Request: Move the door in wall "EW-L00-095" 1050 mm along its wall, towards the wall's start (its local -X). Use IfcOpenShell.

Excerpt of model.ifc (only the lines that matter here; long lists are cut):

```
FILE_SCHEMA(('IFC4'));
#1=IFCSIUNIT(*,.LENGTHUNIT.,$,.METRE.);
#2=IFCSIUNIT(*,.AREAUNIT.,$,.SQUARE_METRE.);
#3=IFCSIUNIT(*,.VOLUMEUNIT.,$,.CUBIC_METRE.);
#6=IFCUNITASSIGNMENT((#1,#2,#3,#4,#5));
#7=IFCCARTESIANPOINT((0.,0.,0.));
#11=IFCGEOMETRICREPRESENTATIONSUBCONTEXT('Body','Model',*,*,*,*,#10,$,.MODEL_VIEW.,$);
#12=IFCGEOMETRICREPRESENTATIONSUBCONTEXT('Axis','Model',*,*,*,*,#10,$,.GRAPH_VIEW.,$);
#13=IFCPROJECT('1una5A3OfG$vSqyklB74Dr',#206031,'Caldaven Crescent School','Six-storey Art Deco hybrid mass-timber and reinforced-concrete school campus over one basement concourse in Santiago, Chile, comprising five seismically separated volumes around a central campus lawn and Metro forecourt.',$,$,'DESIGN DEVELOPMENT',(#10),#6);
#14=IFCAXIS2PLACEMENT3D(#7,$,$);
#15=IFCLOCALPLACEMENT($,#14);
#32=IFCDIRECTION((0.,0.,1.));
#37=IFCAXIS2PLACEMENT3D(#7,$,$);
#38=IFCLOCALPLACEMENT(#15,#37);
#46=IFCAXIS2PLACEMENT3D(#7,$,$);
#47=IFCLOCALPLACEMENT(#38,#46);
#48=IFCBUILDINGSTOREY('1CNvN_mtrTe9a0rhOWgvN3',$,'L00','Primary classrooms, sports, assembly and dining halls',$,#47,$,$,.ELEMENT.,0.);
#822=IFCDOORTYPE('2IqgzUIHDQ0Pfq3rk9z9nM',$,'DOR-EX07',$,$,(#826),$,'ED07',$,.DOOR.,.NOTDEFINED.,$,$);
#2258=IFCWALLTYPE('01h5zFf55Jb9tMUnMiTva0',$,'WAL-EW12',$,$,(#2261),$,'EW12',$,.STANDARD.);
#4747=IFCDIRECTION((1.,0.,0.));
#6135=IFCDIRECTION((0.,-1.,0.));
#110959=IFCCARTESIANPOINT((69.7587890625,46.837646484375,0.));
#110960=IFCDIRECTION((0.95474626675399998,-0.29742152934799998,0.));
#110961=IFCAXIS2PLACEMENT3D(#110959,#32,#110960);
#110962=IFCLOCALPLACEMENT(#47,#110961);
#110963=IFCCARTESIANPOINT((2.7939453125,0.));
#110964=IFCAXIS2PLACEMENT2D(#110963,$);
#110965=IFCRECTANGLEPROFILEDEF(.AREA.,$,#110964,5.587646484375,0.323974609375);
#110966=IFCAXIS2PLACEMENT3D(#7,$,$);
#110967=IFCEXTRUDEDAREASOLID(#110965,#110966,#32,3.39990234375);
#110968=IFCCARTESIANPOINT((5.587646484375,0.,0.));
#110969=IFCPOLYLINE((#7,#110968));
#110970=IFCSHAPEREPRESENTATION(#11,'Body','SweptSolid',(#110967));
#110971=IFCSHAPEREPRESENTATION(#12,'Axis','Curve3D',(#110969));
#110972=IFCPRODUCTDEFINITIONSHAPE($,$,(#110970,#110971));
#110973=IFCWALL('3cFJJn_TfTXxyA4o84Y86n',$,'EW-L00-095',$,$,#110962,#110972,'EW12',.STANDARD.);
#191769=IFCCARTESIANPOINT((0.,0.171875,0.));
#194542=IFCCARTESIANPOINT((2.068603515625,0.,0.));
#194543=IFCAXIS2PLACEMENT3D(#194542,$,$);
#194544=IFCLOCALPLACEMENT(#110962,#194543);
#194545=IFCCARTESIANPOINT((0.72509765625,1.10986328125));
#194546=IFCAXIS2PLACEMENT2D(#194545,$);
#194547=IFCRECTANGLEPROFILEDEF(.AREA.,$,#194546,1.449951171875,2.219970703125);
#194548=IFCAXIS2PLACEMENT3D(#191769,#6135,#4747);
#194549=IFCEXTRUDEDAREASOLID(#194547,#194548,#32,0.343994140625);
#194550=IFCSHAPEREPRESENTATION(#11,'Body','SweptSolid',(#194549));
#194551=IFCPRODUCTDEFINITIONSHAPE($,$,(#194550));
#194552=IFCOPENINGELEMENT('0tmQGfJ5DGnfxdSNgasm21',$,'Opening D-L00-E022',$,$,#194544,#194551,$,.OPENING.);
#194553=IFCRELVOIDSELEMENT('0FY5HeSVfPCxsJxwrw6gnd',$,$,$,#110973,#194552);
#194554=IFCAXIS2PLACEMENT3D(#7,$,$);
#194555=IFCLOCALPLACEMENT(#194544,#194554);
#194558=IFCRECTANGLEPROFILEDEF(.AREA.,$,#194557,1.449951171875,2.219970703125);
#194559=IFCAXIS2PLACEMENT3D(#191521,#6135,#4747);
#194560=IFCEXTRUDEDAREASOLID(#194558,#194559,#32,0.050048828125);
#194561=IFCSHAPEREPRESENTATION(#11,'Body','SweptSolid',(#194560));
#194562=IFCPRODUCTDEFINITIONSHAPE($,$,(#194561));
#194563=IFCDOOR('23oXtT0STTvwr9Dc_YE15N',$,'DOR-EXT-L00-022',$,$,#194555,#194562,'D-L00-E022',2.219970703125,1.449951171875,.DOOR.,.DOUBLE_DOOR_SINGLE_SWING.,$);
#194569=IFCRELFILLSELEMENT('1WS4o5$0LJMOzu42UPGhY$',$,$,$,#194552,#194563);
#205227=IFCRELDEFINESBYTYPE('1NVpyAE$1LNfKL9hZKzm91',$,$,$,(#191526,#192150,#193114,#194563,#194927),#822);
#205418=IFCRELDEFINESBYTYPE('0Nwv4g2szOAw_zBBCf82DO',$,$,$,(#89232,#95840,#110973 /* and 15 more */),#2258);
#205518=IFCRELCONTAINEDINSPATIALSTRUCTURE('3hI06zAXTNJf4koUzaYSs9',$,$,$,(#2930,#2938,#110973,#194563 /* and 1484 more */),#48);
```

```python
import ifcopenshell
import ifcopenshell.api.geometry
import ifcopenshell.util.placement

model = ifcopenshell.open("model.ifc")

door = model.by_guid("23oXtT0STTvwr9Dc_YE15N")
opening = door.FillsVoids[0].RelatingOpeningElement
wall = opening.VoidsElements[0].RelatingBuildingElement

wall_matrix = ifcopenshell.util.placement.get_local_placement(wall.ObjectPlacement)
shift = wall_matrix[:3, 0] * -1.05
before = ifcopenshell.util.placement.get_local_placement(door.ObjectPlacement)[:3, 3].copy()

# The door is placed relative to its opening, so it follows when the opening moves.
matrix = ifcopenshell.util.placement.get_local_placement(opening.ObjectPlacement)
matrix[:3, 3] += shift
ifcopenshell.api.geometry.edit_object_placement(
    model, product=opening, matrix=matrix, is_si=False, should_transform_children=True
)

after = ifcopenshell.util.placement.get_local_placement(door.ObjectPlacement)[:3, 3]
print("door moved by", (after - before).round(3) + 0.0)

model.write("model_v2.ifc")
```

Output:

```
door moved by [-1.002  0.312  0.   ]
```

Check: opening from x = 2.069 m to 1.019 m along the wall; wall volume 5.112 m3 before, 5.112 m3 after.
